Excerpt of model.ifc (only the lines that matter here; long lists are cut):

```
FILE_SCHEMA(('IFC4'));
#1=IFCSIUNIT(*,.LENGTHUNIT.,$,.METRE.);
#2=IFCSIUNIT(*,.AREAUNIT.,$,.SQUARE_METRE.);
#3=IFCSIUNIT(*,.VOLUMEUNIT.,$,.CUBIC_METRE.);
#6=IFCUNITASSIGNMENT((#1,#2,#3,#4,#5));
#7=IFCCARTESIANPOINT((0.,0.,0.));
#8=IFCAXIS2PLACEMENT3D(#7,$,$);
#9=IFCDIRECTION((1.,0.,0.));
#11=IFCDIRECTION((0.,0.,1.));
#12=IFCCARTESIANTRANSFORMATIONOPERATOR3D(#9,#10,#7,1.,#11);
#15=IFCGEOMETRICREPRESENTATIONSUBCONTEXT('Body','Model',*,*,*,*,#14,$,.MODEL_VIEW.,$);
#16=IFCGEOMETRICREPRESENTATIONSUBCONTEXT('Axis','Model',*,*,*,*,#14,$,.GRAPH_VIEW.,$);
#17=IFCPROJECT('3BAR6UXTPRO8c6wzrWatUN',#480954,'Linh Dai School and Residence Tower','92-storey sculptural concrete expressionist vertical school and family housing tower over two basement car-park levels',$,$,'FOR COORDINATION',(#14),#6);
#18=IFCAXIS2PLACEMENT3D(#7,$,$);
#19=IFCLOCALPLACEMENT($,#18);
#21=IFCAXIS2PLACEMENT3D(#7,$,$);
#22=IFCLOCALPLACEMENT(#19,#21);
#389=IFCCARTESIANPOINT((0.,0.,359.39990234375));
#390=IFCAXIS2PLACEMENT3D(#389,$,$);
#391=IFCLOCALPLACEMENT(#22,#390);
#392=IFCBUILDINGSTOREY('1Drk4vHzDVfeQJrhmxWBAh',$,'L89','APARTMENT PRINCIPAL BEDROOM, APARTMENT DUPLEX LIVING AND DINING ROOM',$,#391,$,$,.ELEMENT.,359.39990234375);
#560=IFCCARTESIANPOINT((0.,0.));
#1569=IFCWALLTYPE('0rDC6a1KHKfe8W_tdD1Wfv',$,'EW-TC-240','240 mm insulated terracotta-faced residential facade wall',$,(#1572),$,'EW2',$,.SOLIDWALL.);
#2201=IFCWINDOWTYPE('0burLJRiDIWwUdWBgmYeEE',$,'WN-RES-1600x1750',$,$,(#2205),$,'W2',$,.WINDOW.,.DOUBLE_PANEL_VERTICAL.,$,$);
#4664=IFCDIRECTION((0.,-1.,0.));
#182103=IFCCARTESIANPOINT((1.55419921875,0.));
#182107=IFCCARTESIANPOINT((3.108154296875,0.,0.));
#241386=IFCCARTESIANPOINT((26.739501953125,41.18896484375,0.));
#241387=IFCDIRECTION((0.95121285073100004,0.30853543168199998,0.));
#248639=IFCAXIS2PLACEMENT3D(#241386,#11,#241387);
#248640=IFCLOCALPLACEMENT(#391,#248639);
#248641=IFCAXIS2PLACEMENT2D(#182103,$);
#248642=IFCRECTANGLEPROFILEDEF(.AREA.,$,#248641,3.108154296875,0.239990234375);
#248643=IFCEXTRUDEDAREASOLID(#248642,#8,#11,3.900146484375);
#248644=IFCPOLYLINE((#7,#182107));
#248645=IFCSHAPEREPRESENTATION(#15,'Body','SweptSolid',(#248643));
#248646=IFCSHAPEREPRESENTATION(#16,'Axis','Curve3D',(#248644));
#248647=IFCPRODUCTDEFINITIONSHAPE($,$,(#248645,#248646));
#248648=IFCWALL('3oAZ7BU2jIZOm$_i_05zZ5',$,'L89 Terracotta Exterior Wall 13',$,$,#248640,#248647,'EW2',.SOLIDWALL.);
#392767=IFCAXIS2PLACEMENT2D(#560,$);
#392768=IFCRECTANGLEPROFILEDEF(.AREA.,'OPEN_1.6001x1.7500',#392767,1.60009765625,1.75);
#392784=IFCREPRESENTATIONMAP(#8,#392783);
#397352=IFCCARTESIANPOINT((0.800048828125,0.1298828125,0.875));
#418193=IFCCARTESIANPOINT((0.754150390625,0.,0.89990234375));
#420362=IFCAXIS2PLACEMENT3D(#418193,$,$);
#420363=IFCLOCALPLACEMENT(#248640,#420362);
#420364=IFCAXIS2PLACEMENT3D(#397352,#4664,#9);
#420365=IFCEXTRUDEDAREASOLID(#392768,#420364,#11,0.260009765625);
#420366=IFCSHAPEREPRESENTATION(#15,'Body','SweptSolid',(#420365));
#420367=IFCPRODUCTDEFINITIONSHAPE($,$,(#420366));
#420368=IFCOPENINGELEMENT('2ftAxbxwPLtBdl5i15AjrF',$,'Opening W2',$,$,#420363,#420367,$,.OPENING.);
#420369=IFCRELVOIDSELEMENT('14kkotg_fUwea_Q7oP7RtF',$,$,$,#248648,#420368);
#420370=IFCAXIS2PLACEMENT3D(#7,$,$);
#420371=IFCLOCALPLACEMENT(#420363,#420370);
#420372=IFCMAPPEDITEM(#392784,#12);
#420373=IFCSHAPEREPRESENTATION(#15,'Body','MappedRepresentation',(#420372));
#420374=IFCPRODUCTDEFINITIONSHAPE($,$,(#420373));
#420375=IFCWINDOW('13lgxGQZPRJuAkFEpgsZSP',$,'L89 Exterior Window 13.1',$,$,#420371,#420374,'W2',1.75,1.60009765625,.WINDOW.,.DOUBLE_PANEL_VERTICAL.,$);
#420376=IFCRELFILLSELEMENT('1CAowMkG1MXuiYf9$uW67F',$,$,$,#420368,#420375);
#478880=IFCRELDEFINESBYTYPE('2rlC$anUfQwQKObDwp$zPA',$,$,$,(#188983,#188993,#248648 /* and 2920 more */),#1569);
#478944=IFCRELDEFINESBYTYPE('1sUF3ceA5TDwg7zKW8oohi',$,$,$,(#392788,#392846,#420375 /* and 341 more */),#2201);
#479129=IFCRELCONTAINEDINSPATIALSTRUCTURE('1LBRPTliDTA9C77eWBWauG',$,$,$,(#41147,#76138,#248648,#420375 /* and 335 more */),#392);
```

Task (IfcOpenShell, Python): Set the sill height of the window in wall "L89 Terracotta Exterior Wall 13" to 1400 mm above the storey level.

```python
import numpy as np
import ifcopenshell
import ifcopenshell.api.geometry
import ifcopenshell.geom
import ifcopenshell.util.element
import ifcopenshell.util.placement
import ifcopenshell.util.shape
import ifcopenshell.util.unit

model = ifcopenshell.open("model.ifc")
unit_scale = ifcopenshell.util.unit.calculate_unit_scale(model)

window = model.by_guid("13lgxGQZPRJuAkFEpgsZSP")
opening = window.FillsVoids[0].RelatingOpeningElement
storey = ifcopenshell.util.element.get_container(window, ifc_class="IfcBuildingStorey")
level = ifcopenshell.util.placement.get_local_placement(storey.ObjectPlacement)[2, 3]

# The opening's origin need not be at the sill, so measure its lowest point.
shape = ifcopenshell.geom.create_shape(ifcopenshell.geom.settings(), opening)
bottom = ifcopenshell.util.shape.get_shape_bottom_elevation(shape, shape.geometry) / unit_scale
dz = level + 1.4 - bottom

shift = np.array([0.0, 0.0, dz])
# The window is placed relative to its opening, so it follows when the opening moves.
matrix = ifcopenshell.util.placement.get_local_placement(opening.ObjectPlacement)
matrix[:3, 3] += shift
ifcopenshell.api.geometry.edit_object_placement(
    model, product=opening, matrix=matrix, is_si=False, should_transform_children=True
)

print(f"moved by {dz * unit_scale:+.3f} m")

model.write("model_rev.ifc")
```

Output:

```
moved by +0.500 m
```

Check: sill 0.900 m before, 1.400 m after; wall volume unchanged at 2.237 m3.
